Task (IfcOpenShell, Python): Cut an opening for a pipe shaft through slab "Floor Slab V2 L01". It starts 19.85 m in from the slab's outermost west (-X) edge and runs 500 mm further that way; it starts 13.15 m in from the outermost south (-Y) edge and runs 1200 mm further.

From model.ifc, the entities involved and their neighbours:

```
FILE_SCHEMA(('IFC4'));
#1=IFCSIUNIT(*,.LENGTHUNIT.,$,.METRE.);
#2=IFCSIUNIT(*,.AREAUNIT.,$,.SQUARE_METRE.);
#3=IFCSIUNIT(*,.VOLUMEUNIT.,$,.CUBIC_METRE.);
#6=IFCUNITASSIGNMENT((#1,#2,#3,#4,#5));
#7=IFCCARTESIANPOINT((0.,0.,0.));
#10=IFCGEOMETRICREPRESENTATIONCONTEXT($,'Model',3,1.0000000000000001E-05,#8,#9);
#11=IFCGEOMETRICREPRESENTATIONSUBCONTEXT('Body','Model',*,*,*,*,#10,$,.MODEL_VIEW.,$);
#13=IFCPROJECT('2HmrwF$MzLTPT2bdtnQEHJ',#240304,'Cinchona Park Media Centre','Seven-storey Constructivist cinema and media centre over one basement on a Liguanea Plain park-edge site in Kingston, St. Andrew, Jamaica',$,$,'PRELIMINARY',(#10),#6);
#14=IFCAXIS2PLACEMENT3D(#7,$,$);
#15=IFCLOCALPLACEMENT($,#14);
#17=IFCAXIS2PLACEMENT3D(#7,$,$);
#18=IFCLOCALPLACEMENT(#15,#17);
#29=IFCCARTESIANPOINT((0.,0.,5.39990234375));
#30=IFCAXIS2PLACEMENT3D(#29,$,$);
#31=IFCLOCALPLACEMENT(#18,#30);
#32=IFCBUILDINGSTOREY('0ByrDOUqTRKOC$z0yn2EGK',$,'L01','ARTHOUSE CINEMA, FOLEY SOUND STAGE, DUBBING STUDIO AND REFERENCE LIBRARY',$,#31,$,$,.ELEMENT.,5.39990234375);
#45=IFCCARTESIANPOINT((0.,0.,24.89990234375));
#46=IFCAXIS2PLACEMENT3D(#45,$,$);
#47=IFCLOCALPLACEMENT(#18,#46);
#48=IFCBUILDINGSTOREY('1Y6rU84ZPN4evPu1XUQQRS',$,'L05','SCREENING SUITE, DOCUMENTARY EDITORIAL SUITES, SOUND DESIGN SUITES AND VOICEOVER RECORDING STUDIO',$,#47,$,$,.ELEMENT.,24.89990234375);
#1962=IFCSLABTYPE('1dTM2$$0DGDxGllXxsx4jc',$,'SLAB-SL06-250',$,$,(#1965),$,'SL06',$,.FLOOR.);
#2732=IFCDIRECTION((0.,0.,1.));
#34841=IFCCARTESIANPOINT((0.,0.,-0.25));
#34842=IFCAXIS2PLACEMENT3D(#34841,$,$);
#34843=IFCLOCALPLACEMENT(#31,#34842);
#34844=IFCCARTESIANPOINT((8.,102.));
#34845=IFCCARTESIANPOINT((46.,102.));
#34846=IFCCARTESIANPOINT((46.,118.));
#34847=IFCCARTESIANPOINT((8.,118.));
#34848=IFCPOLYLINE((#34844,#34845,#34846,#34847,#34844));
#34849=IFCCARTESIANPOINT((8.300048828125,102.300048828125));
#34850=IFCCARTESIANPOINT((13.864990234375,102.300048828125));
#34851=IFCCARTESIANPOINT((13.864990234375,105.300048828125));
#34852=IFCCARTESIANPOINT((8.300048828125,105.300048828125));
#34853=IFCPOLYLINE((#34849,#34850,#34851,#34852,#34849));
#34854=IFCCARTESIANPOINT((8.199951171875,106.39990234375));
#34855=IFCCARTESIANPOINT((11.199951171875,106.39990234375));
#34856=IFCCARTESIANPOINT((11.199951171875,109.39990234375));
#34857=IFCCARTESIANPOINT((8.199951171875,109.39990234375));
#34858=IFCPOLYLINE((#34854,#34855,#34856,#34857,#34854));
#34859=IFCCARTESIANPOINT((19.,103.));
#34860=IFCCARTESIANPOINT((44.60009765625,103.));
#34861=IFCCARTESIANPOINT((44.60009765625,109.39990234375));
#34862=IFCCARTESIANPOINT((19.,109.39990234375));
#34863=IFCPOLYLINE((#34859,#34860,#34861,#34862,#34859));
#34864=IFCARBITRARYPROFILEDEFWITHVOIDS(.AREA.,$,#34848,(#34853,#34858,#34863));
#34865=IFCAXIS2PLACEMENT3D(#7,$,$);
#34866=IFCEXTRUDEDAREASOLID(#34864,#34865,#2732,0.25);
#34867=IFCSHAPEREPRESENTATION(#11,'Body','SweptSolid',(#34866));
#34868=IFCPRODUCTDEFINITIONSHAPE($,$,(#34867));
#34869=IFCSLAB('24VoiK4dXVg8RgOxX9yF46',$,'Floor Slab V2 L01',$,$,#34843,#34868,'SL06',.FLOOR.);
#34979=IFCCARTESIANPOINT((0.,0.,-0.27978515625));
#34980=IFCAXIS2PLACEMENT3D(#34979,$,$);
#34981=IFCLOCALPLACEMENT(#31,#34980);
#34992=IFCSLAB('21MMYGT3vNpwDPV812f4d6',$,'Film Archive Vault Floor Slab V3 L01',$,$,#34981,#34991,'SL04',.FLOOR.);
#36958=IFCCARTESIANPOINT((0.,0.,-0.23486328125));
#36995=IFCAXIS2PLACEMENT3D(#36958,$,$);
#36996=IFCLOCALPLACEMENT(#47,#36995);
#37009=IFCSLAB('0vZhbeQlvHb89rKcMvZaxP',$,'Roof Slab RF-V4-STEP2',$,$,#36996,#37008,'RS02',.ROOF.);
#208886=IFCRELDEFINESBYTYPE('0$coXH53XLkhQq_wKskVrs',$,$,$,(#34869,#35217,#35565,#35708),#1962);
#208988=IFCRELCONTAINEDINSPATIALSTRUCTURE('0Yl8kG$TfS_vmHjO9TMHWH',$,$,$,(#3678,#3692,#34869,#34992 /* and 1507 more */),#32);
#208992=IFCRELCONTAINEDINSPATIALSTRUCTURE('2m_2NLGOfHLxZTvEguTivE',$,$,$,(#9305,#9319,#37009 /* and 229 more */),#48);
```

```python
import numpy as np
import ifcopenshell
import ifcopenshell.api.feature
import ifcopenshell.api.geometry
import ifcopenshell.api.root
import ifcopenshell.geom
import ifcopenshell.util.placement
import ifcopenshell.util.representation
import ifcopenshell.util.shape
import ifcopenshell.util.unit

model = ifcopenshell.open("model.ifc")
unit_scale = ifcopenshell.util.unit.calculate_unit_scale(model)
settings = ifcopenshell.geom.settings()


def volume(element):
    """Net volume in cubic metres, openings subtracted."""
    shape = ifcopenshell.geom.create_shape(settings, element)
    return ifcopenshell.util.shape.get_volume(shape.geometry)


slab = model.by_guid("24VoiK4dXVg8RgOxX9yF46")
before = volume(slab)

# Extent in the slab's own axes, in metres. The edges named are its -X and -Y sides.
slab_shape = ifcopenshell.geom.create_shape(settings, slab)
vertices = ifcopenshell.util.shape.get_vertices(slab_shape.geometry)
x_min, y_min, bottom = vertices.min(axis=0)
top = vertices[:, 2].max()

opening = ifcopenshell.api.root.create_entity(model, ifc_class="IfcOpeningElement", name="Pipe shaft opening", predefined_type="OPENING")
context = ifcopenshell.util.representation.get_context(model, "Model", "Body", "MODEL_VIEW")
width, depth = 0.5, 1.2
outline = [(0.0, 0.0), (width, 0.0), (width, depth), (0.0, depth), (0.0, 0.0)]
# Overshoot both faces by 50 mm so the cut is clean.
shape = ifcopenshell.api.geometry.add_slab_representation(
    model, context=context, depth=top - bottom + 0.1, polyline=outline
)
ifcopenshell.api.geometry.assign_representation(model, product=opening, representation=shape)

matrix = ifcopenshell.util.placement.get_local_placement(slab.ObjectPlacement)
matrix[:, 3] = matrix @ np.append(np.array([x_min + 19.85, y_min + 13.15, bottom - 0.05]) / unit_scale, 1.0)
ifcopenshell.api.geometry.edit_object_placement(model, product=opening, matrix=matrix, is_si=False)
ifcopenshell.api.feature.add_feature(model, feature=opening, element=slab)

after = volume(slab)

print(f"slab volume {before:.3f} -> {after:.3f} m3")

model.write("model_updated.ifc")
```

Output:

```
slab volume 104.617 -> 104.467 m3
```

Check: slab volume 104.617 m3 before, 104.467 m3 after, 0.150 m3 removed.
